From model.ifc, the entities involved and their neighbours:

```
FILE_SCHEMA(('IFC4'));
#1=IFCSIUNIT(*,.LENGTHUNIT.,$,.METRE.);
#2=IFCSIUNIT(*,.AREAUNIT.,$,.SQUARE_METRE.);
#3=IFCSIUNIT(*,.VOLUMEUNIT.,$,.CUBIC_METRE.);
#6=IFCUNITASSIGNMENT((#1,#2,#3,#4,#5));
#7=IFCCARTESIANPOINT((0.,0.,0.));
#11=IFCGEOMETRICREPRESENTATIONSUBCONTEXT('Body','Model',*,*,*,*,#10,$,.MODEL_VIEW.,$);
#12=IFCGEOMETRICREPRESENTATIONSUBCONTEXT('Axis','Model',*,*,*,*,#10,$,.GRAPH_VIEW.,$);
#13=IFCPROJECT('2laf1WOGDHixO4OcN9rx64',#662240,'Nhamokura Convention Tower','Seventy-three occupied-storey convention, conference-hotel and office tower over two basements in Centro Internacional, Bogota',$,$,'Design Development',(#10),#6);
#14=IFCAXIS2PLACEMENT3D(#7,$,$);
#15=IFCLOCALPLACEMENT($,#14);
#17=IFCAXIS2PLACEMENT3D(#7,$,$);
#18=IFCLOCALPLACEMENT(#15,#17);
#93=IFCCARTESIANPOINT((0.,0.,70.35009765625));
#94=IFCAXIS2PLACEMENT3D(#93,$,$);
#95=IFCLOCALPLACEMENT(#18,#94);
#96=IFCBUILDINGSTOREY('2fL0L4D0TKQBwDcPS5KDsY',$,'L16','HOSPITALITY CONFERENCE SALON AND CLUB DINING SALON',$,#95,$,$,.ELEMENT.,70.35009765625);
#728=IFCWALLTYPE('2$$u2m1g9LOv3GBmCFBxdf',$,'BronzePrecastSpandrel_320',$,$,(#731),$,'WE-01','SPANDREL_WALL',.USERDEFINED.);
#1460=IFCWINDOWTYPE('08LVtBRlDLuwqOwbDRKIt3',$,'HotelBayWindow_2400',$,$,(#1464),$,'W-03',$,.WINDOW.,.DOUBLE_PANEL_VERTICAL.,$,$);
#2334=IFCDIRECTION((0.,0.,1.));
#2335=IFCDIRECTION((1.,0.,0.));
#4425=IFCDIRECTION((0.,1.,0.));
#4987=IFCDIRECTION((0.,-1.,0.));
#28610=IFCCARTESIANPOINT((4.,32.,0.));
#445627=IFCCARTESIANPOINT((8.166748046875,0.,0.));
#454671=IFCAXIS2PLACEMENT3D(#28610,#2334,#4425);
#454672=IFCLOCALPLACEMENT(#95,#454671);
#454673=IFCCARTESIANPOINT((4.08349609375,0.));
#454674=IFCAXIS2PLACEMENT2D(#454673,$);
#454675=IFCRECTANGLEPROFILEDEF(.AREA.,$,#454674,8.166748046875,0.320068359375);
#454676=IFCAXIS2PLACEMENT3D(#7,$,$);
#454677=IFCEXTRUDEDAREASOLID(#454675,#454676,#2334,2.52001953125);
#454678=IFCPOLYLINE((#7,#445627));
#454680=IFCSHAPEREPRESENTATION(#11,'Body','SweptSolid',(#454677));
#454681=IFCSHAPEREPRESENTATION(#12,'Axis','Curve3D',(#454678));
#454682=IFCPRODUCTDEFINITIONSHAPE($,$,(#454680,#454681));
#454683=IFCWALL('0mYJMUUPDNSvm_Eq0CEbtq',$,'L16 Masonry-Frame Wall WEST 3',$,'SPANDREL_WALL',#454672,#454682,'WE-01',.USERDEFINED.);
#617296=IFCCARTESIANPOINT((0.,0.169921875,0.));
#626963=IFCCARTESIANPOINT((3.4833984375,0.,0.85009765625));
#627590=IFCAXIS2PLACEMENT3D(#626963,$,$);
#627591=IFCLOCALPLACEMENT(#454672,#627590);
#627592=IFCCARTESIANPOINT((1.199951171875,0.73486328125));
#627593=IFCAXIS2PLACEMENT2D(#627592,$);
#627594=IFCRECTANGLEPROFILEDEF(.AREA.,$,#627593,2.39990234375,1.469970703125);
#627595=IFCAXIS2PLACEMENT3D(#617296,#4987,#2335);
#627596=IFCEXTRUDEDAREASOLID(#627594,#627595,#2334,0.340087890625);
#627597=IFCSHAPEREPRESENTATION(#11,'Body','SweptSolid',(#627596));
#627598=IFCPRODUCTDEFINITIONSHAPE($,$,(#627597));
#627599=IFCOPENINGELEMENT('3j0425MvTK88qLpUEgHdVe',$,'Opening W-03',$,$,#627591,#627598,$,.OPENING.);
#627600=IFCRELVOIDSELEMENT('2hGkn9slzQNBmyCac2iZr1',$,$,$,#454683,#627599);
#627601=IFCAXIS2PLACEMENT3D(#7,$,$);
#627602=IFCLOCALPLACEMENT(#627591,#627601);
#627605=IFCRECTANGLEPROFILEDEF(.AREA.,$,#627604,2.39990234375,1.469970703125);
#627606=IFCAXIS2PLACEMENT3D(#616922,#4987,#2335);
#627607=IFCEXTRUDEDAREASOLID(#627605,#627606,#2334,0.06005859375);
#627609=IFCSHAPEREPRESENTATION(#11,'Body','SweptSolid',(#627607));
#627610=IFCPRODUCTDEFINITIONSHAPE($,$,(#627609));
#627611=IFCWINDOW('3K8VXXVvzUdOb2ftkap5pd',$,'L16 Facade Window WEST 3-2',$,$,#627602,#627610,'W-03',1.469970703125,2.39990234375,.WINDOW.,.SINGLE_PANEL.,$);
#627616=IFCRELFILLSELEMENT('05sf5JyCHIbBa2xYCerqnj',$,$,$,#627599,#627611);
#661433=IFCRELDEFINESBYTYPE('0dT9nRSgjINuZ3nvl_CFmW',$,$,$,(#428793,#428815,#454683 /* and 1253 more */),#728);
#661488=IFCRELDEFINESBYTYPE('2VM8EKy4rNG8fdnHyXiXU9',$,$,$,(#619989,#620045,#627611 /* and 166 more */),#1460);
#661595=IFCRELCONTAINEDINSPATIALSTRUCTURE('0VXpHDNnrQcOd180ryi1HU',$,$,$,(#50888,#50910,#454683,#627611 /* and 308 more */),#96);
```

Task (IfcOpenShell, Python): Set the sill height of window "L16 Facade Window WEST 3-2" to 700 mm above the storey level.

```python
import numpy as np
import ifcopenshell
import ifcopenshell.api.geometry
import ifcopenshell.geom
import ifcopenshell.util.element
import ifcopenshell.util.placement
import ifcopenshell.util.shape
import ifcopenshell.util.unit

model = ifcopenshell.open("model.ifc")
unit_scale = ifcopenshell.util.unit.calculate_unit_scale(model)

window = model.by_guid("3K8VXXVvzUdOb2ftkap5pd")
opening = window.FillsVoids[0].RelatingOpeningElement
storey = ifcopenshell.util.element.get_container(window, ifc_class="IfcBuildingStorey")
level = ifcopenshell.util.placement.get_local_placement(storey.ObjectPlacement)[2, 3]

# The opening's origin need not be at the sill, so measure its lowest point.
shape = ifcopenshell.geom.create_shape(ifcopenshell.geom.settings(), opening)
bottom = ifcopenshell.util.shape.get_shape_bottom_elevation(shape, shape.geometry) / unit_scale
dz = level + 0.7 / unit_scale - bottom

shift = np.array([0.0, 0.0, dz])
# The window is placed relative to its opening, so it follows when the opening moves.
matrix = ifcopenshell.util.placement.get_local_placement(opening.ObjectPlacement)
matrix[:3, 3] += shift
ifcopenshell.api.geometry.edit_object_placement(
    model, product=opening, matrix=matrix, is_si=False, should_transform_children=True
)

print(f"moved by {dz * unit_scale:+.3f} m")

model.write("model_v2.ifc")
```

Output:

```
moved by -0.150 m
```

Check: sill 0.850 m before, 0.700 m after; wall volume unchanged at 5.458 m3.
